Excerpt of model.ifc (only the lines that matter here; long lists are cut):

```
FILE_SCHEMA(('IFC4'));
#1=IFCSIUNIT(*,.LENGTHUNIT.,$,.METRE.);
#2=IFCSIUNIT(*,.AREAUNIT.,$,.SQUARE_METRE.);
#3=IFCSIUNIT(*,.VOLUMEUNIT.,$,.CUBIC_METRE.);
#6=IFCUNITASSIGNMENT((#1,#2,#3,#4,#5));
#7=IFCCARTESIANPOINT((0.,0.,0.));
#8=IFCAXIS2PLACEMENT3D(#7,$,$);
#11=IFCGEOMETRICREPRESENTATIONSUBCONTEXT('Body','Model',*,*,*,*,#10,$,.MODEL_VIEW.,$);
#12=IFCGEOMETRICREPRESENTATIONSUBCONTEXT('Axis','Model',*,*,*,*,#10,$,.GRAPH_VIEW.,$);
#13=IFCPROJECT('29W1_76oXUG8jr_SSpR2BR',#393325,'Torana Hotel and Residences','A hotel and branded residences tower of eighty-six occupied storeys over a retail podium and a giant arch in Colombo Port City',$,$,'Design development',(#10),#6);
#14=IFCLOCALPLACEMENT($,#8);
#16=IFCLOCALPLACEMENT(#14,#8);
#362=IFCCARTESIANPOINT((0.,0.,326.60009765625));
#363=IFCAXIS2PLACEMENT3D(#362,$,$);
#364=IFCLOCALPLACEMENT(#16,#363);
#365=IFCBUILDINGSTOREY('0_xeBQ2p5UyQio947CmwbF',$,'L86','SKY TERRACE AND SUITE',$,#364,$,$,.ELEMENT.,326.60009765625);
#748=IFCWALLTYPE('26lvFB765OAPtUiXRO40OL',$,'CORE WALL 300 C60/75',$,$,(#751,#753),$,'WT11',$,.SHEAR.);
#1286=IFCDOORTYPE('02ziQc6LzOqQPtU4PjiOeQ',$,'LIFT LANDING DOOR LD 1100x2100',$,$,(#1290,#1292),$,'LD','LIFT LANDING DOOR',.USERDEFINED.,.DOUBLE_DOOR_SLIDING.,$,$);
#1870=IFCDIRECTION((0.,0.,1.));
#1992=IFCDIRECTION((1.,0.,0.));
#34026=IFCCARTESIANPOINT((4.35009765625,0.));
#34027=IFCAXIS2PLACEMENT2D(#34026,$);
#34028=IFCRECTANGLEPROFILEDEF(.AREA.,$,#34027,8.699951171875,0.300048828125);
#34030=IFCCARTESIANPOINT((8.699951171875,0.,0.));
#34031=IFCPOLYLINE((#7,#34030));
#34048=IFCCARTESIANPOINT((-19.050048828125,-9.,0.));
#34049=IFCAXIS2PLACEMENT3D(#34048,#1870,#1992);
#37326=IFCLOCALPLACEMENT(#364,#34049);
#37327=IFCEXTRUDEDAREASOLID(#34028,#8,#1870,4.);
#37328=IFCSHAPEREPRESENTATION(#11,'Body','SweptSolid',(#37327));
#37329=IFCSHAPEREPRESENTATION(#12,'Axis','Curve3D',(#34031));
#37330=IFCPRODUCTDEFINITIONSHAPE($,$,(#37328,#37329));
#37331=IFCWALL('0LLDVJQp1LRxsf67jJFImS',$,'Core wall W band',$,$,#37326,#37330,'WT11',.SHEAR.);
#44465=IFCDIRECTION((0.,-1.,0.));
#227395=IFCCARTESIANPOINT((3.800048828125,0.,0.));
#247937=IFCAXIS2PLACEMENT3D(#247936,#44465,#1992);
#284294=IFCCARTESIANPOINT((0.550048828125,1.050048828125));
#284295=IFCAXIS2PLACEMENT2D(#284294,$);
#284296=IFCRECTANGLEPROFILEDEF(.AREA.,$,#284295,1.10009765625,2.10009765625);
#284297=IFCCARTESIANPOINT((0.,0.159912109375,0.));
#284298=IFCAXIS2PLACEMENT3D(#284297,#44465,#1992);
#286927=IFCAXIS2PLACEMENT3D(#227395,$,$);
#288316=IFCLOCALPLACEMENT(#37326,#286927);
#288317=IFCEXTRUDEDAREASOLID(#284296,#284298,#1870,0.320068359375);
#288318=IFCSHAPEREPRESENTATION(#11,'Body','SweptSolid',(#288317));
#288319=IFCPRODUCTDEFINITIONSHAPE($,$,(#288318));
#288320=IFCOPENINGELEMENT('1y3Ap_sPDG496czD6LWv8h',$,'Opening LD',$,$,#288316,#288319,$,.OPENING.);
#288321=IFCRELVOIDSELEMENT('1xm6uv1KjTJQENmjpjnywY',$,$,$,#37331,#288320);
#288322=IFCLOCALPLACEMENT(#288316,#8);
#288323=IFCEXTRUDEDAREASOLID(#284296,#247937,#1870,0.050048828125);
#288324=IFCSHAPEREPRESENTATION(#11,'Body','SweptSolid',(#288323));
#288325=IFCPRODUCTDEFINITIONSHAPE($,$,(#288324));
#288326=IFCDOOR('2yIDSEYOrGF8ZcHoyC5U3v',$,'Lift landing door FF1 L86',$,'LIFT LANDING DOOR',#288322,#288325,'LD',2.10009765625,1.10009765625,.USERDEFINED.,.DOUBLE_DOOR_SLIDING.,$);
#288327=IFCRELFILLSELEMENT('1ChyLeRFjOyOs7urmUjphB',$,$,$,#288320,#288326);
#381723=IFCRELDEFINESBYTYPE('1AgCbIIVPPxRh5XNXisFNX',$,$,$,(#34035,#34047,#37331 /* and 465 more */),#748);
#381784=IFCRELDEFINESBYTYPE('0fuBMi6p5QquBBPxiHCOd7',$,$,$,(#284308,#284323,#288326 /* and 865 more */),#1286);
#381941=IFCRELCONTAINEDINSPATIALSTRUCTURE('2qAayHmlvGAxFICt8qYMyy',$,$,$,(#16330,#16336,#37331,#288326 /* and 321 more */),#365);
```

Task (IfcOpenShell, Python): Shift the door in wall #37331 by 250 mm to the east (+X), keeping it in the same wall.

```python
import ifcopenshell
import ifcopenshell.api.geometry
import ifcopenshell.util.placement
import ifcopenshell.util.unit

model = ifcopenshell.open("model.ifc")
unit_scale = ifcopenshell.util.unit.calculate_unit_scale(model)

door = model.by_guid("2yIDSEYOrGF8ZcHoyC5U3v")
opening = door.FillsVoids[0].RelatingOpeningElement
wall = opening.VoidsElements[0].RelatingBuildingElement

wall_matrix = ifcopenshell.util.placement.get_local_placement(wall.ObjectPlacement)
shift = wall_matrix[:3, 0] * 0.25 / unit_scale
before = ifcopenshell.util.placement.get_local_placement(door.ObjectPlacement)[:3, 3].copy()

# The door is placed relative to its opening, so it follows when the opening moves.
matrix = ifcopenshell.util.placement.get_local_placement(opening.ObjectPlacement)
matrix[:3, 3] += shift
ifcopenshell.api.geometry.edit_object_placement(
    model, product=opening, matrix=matrix, is_si=False, should_transform_children=True
)

after = ifcopenshell.util.placement.get_local_placement(door.ObjectPlacement)[:3, 3]
print("door moved by", (after - before).round(3) + 0.0)

model.write("model_v2.ifc")
```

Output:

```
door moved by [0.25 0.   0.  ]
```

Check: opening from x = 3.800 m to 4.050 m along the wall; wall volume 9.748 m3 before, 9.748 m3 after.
